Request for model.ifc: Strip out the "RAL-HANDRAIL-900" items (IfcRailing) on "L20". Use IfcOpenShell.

First a look at what the model holds.

```python
import ifcopenshell
import ifcopenshell.util.element

model = ifcopenshell.open("model.ifc")
print(model.schema)
storey = next(s for s in model.by_type("IfcBuildingStorey") if s.Name == "L20")
railings = [e for e in ifcopenshell.util.element.get_decomposition(storey) if e.is_a("IfcRailing")]
seen = {}
for e in railings:
    element_type = ifcopenshell.util.element.get_type(e)
    name = element_type.Name if element_type not in (None, e) else None
    seen[name] = seen.get(name, 0) + 1
for name, count in sorted(seen.items(), key=str):
    print(count, "x", name)
```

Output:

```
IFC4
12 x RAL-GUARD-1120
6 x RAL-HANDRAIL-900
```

```python
import ifcopenshell
import ifcopenshell.api.root
import ifcopenshell.util.element

model = ifcopenshell.open("model.ifc")

storey = next(s for s in model.by_type("IfcBuildingStorey") if s.Name == "L20")
railings = [e for e in ifcopenshell.util.element.get_decomposition(storey) if e.is_a("IfcRailing")]
targets = [e for e in railings if (t := ifcopenshell.util.element.get_type(e)) not in (None, e) and t.Name == "RAL-HANDRAIL-900"]

for e in targets:
    ifcopenshell.api.root.remove_product(model, product=e)
print(len(targets), "removed")

model.write("model_updated.ifc")
```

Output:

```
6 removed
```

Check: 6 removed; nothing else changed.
